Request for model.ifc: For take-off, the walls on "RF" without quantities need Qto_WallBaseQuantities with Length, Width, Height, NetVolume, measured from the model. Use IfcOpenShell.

First a look at what the model holds.

```python
import ifcopenshell
import ifcopenshell.util.element
import ifcopenshell.util.unit

model = ifcopenshell.open("model.ifc")
print(model.schema)
for unit_type in ("LENGTHUNIT", "AREAUNIT", "VOLUMEUNIT"):
    print(unit_type, ifcopenshell.util.unit.calculate_unit_scale(model, unit_type))
storey = next(s for s in model.by_type("IfcBuildingStorey") if s.Name == "RF")
walls = [e for e in ifcopenshell.util.element.get_decomposition(storey) if e.is_a("IfcWall")]
for e in sorted(walls, key=lambda e: e.id()):
    print(e.id(), e.is_a(), e.Name, list(ifcopenshell.util.element.get_psets(e, qtos_only=True)), sep=" | ")
```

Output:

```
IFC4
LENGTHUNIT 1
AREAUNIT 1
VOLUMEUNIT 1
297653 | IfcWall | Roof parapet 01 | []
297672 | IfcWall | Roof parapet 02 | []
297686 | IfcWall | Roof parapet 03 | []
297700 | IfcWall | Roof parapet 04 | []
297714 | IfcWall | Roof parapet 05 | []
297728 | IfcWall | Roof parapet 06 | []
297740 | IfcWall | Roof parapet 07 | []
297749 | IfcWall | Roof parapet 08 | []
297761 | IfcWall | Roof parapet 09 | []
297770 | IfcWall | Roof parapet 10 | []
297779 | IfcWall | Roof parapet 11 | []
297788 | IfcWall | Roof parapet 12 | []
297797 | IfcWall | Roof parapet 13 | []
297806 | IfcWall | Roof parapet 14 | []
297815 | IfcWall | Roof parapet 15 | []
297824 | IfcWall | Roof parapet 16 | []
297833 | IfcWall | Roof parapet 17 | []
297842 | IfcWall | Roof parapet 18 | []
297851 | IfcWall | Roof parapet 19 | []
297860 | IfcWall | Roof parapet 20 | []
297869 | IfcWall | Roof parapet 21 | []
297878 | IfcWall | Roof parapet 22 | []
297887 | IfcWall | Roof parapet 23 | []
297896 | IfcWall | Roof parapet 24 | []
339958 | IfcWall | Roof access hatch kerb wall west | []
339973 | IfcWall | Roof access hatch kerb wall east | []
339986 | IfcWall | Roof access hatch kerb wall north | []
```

```python
import ifcopenshell
import ifcopenshell.api.pset
import ifcopenshell.geom
import ifcopenshell.util.element
import ifcopenshell.util.shape
import ifcopenshell.util.unit

model = ifcopenshell.open("model.ifc")
unit_scale = ifcopenshell.util.unit.calculate_unit_scale(model)
volume_scale = ifcopenshell.util.unit.calculate_unit_scale(model, "VOLUMEUNIT")
settings = ifcopenshell.geom.settings()

storey = next(s for s in model.by_type("IfcBuildingStorey") if s.Name == "RF")
walls = [e for e in ifcopenshell.util.element.get_decomposition(storey) if e.is_a("IfcWall")]

for e in sorted(walls, key=lambda e: e.id()):
    if ifcopenshell.util.element.get_psets(e, qtos_only=True, should_inherit=False):
        continue
    # Geometry comes back in metres, in the element's own axes.
    shape = ifcopenshell.geom.create_shape(settings, e)
    values = {
        "Length": ifcopenshell.util.shape.get_x(shape.geometry) / unit_scale,
        "Width": ifcopenshell.util.shape.get_y(shape.geometry) / unit_scale,
        "Height": ifcopenshell.util.shape.get_z(shape.geometry) / unit_scale,
        "NetVolume": ifcopenshell.util.shape.get_volume(shape.geometry) / volume_scale,
    }
    qto = ifcopenshell.api.pset.add_qto(model, product=e, name="Qto_WallBaseQuantities")
    ifcopenshell.api.pset.edit_qto(model, qto=qto, properties=values)
    print(e.id(), {k: round(v, 3) for k, v in values.items()})

model.write("model_rev.ifc")
```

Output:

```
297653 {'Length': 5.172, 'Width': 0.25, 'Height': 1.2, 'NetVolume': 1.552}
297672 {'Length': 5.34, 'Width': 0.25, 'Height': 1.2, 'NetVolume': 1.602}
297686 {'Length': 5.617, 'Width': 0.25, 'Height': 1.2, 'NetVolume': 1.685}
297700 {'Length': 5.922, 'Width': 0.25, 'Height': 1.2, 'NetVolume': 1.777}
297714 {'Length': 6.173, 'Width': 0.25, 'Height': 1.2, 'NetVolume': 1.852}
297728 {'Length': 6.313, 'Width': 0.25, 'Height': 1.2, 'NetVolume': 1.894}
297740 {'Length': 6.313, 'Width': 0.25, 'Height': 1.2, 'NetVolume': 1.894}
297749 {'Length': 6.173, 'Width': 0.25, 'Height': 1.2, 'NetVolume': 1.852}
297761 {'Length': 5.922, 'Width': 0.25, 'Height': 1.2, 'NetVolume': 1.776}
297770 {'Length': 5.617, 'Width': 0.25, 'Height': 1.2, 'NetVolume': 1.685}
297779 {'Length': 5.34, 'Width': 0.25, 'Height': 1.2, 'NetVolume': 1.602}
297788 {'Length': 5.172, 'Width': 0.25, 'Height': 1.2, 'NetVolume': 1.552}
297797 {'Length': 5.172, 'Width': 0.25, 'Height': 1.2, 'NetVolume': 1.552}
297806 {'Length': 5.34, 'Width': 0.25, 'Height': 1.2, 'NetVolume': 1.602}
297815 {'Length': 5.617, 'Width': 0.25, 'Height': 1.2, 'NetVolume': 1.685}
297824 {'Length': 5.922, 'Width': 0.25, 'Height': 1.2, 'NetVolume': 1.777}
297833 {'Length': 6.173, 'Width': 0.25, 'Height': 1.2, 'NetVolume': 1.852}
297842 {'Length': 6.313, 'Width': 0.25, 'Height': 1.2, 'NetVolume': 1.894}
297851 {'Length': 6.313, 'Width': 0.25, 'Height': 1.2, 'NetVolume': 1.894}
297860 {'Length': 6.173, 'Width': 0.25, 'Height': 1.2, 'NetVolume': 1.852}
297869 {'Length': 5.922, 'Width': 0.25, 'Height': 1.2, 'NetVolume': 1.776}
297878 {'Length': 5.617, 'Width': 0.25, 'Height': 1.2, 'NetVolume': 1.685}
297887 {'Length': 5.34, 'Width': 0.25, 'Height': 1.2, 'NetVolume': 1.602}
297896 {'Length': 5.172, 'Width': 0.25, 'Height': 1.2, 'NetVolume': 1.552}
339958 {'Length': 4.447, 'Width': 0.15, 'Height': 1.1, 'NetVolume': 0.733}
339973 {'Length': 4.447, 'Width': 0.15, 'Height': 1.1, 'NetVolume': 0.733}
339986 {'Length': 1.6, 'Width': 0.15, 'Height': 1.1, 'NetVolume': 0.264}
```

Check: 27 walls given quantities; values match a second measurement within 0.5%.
